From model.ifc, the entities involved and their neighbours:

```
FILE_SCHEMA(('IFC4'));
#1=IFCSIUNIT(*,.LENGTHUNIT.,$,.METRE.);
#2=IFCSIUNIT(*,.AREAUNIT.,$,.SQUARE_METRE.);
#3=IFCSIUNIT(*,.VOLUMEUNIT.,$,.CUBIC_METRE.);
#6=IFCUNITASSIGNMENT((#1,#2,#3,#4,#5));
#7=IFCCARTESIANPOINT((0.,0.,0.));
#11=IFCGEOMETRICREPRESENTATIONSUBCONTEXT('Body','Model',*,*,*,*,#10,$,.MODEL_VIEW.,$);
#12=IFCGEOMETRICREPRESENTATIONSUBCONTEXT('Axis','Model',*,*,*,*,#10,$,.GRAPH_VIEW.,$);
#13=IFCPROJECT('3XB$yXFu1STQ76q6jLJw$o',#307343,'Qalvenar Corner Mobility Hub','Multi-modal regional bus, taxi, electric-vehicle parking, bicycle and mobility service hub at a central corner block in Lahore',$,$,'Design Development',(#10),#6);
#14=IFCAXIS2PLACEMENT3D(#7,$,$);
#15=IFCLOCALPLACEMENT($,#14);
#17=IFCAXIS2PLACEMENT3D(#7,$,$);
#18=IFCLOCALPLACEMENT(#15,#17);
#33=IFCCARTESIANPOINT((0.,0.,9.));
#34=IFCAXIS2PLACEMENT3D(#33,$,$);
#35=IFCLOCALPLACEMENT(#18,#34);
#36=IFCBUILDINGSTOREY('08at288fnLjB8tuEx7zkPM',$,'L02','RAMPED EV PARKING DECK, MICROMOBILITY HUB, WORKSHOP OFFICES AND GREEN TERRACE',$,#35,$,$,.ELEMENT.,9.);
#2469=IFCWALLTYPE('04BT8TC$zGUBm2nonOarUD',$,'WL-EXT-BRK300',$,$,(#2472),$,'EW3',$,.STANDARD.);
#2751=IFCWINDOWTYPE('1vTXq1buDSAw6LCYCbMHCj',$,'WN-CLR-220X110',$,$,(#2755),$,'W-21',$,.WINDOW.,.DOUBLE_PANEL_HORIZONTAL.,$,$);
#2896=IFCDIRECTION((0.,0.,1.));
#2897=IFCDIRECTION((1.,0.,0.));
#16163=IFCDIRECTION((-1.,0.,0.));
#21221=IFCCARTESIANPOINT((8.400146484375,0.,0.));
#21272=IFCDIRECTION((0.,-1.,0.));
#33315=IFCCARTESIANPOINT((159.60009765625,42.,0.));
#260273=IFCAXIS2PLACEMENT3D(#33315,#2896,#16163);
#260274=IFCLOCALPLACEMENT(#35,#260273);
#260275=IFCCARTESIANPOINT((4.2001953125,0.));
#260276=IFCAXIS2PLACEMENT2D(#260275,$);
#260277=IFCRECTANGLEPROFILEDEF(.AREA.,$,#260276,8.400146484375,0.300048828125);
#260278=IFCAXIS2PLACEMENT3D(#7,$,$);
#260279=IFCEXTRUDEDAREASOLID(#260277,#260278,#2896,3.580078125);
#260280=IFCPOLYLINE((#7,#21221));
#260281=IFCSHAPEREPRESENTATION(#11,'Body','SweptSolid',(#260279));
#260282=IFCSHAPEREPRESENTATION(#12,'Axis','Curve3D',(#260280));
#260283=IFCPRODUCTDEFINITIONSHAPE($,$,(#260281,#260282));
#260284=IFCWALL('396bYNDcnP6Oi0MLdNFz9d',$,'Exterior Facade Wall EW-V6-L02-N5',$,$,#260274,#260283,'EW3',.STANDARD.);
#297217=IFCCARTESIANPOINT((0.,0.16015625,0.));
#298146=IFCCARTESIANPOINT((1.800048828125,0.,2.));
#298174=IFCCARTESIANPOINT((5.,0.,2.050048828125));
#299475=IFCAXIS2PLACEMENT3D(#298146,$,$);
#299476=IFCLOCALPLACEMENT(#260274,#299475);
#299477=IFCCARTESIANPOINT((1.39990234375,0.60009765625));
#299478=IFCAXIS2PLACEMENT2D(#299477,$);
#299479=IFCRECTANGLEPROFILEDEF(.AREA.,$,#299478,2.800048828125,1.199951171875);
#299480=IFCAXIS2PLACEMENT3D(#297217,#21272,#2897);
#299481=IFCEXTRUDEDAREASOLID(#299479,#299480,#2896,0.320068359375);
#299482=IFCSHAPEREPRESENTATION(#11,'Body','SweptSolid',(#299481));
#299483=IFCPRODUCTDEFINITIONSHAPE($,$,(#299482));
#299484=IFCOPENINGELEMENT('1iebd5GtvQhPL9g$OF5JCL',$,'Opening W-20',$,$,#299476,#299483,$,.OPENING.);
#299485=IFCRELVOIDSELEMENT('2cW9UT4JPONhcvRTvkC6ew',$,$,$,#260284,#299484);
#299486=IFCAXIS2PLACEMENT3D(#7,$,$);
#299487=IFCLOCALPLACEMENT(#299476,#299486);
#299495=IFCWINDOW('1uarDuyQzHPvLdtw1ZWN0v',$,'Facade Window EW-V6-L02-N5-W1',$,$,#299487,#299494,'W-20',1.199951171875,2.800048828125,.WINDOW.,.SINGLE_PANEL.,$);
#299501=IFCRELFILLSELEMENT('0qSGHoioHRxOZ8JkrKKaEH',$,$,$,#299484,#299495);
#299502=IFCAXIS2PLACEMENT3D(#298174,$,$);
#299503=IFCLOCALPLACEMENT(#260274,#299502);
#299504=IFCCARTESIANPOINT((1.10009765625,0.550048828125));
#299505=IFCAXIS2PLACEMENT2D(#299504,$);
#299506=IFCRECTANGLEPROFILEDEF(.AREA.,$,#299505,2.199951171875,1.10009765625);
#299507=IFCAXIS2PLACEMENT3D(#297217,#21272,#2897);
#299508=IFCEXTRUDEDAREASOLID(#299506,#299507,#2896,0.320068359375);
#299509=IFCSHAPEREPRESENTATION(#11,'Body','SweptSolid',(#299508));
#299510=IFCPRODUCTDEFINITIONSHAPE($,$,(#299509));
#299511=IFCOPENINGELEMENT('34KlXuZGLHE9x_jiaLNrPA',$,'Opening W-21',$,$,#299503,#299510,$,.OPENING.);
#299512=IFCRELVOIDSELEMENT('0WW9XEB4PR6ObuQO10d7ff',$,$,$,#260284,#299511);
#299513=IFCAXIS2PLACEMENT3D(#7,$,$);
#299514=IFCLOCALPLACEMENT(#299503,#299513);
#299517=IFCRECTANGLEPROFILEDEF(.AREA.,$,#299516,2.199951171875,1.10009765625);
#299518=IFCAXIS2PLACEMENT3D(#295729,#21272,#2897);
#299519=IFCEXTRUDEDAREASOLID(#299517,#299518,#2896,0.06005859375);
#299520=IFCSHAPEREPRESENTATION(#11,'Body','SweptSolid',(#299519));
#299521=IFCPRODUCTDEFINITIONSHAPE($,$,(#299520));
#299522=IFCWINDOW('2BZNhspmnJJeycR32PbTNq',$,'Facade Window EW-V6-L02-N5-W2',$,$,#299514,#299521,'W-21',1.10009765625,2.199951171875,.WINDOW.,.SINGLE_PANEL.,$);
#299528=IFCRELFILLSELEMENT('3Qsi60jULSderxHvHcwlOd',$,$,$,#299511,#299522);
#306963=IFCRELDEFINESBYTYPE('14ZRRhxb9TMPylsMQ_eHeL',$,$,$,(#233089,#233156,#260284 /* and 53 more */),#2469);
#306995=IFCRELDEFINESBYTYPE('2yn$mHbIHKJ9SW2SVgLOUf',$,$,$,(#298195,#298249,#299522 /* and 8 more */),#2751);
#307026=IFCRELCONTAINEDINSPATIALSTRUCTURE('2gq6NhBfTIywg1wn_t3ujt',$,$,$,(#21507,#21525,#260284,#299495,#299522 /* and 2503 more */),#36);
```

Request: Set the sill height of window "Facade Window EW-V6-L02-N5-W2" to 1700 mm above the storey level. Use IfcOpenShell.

```python
import numpy as np
import ifcopenshell
import ifcopenshell.api.geometry
import ifcopenshell.geom
import ifcopenshell.util.element
import ifcopenshell.util.placement
import ifcopenshell.util.shape
import ifcopenshell.util.unit

model = ifcopenshell.open("model.ifc")
unit_scale = ifcopenshell.util.unit.calculate_unit_scale(model)

window = model.by_id(299522)
opening = window.FillsVoids[0].RelatingOpeningElement
storey = ifcopenshell.util.element.get_container(window, ifc_class="IfcBuildingStorey")
level = ifcopenshell.util.placement.get_local_placement(storey.ObjectPlacement)[2, 3]

# The opening's origin need not be at the sill, so measure its lowest point.
shape = ifcopenshell.geom.create_shape(ifcopenshell.geom.settings(), opening)
bottom = ifcopenshell.util.shape.get_shape_bottom_elevation(shape, shape.geometry) / unit_scale
dz = level + 1.7 - bottom

shift = np.array([0.0, 0.0, dz])
# The window is placed relative to its opening, so it follows when the opening moves.
matrix = ifcopenshell.util.placement.get_local_placement(opening.ObjectPlacement)
matrix[:3, 3] += shift
ifcopenshell.api.geometry.edit_object_placement(
    model, product=opening, matrix=matrix, is_si=False, should_transform_children=True
)

print(f"moved by {dz * unit_scale:+.3f} m")

model.write("model_edited.ifc")
```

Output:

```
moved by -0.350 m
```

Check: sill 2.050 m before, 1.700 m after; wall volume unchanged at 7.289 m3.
